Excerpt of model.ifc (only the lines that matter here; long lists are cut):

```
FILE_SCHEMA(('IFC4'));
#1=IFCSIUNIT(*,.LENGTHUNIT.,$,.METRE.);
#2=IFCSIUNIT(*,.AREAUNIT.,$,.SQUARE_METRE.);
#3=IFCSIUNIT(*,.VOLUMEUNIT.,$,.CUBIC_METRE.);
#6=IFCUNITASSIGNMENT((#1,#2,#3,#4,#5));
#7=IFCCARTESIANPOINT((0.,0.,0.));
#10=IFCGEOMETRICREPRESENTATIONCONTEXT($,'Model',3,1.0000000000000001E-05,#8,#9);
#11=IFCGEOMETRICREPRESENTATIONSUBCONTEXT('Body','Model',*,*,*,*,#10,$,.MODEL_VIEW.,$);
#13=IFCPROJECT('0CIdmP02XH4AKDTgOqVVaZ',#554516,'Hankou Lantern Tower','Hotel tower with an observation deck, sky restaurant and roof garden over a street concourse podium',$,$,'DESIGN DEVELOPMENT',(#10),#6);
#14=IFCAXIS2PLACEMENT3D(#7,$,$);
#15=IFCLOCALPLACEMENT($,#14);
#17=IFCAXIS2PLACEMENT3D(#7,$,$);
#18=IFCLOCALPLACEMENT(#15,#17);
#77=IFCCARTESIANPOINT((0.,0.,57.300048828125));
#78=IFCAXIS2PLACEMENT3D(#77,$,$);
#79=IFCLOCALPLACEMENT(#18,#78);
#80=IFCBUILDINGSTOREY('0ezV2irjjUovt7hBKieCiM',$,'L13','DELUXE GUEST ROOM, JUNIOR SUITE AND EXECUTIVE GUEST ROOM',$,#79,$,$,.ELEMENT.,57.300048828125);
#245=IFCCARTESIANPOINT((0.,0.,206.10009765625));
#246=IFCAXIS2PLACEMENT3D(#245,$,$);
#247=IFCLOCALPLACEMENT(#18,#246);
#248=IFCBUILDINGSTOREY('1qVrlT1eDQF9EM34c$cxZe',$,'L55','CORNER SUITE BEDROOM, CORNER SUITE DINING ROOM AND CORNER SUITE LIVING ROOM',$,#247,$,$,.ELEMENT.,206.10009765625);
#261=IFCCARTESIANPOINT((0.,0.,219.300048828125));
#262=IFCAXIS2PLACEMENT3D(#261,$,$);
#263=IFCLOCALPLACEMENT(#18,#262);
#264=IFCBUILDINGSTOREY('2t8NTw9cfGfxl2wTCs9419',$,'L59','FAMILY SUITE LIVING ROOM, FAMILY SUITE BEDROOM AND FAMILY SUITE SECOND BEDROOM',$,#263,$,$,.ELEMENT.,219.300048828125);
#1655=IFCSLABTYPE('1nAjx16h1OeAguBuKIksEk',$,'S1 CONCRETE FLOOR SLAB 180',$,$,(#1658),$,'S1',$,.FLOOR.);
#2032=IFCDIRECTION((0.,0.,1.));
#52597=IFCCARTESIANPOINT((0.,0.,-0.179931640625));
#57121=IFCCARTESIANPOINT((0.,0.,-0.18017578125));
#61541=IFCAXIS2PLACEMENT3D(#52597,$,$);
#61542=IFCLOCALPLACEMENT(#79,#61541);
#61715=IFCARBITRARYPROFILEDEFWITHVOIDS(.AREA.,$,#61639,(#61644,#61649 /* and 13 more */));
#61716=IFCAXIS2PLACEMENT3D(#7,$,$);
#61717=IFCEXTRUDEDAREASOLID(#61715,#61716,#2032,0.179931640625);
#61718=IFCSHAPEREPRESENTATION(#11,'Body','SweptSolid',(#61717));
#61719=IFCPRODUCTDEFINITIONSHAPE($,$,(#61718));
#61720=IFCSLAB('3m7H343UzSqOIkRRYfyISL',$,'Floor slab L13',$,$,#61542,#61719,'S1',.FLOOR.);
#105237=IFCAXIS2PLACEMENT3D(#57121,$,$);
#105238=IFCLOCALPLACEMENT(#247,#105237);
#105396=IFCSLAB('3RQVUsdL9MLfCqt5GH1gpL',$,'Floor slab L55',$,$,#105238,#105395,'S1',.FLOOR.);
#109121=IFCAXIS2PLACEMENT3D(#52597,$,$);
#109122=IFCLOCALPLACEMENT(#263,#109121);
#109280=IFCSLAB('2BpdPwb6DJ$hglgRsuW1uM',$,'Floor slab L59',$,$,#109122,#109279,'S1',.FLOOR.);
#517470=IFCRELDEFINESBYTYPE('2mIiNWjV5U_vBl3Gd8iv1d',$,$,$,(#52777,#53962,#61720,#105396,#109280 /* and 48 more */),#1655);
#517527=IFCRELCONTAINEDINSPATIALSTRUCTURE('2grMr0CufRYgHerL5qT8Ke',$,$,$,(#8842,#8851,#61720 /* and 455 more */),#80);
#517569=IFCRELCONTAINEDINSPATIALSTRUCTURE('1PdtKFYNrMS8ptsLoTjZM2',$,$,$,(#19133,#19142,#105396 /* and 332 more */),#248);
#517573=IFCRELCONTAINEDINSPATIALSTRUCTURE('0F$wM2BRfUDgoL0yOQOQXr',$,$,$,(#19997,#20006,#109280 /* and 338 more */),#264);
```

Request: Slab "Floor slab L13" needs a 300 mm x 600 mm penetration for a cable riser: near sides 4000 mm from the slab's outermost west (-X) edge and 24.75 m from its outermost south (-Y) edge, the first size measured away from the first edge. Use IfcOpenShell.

```python
import numpy as np
import ifcopenshell
import ifcopenshell.api.feature
import ifcopenshell.api.geometry
import ifcopenshell.api.root
import ifcopenshell.geom
import ifcopenshell.util.placement
import ifcopenshell.util.representation
import ifcopenshell.util.shape
import ifcopenshell.util.unit

model = ifcopenshell.open("model.ifc")
unit_scale = ifcopenshell.util.unit.calculate_unit_scale(model)
settings = ifcopenshell.geom.settings()


def volume(element):
    """Net volume in cubic metres, openings subtracted."""
    shape = ifcopenshell.geom.create_shape(settings, element)
    return ifcopenshell.util.shape.get_volume(shape.geometry)


slab = model.by_guid("3m7H343UzSqOIkRRYfyISL")
before = volume(slab)

# Extent in the slab's own axes, in metres. The edges named are its -X and -Y sides.
slab_shape = ifcopenshell.geom.create_shape(settings, slab)
vertices = ifcopenshell.util.shape.get_vertices(slab_shape.geometry)
x_min, y_min, bottom = vertices.min(axis=0)
top = vertices[:, 2].max()

opening = ifcopenshell.api.root.create_entity(model, ifc_class="IfcOpeningElement", name="Cable riser opening", predefined_type="OPENING")
context = ifcopenshell.util.representation.get_context(model, "Model", "Body", "MODEL_VIEW")
width, depth = 0.3, 0.6
outline = [(0.0, 0.0), (width, 0.0), (width, depth), (0.0, depth), (0.0, 0.0)]
# Overshoot both faces by 50 mm so the cut is clean.
shape = ifcopenshell.api.geometry.add_slab_representation(
    model, context=context, depth=top - bottom + 0.1, polyline=outline
)
ifcopenshell.api.geometry.assign_representation(model, product=opening, representation=shape)

matrix = ifcopenshell.util.placement.get_local_placement(slab.ObjectPlacement)
matrix[:, 3] = matrix @ np.append(np.array([x_min + 4, y_min + 24.75, bottom - 0.05]) / unit_scale, 1.0)
ifcopenshell.api.geometry.edit_object_placement(model, product=opening, matrix=matrix, is_si=False)
ifcopenshell.api.feature.add_feature(model, feature=opening, element=slab)

after = volume(slab)

print(f"slab volume {before:.3f} -> {after:.3f} m3")

model.write("model_updated.ifc")
```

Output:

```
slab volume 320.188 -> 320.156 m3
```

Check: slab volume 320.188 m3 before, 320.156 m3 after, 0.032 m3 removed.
